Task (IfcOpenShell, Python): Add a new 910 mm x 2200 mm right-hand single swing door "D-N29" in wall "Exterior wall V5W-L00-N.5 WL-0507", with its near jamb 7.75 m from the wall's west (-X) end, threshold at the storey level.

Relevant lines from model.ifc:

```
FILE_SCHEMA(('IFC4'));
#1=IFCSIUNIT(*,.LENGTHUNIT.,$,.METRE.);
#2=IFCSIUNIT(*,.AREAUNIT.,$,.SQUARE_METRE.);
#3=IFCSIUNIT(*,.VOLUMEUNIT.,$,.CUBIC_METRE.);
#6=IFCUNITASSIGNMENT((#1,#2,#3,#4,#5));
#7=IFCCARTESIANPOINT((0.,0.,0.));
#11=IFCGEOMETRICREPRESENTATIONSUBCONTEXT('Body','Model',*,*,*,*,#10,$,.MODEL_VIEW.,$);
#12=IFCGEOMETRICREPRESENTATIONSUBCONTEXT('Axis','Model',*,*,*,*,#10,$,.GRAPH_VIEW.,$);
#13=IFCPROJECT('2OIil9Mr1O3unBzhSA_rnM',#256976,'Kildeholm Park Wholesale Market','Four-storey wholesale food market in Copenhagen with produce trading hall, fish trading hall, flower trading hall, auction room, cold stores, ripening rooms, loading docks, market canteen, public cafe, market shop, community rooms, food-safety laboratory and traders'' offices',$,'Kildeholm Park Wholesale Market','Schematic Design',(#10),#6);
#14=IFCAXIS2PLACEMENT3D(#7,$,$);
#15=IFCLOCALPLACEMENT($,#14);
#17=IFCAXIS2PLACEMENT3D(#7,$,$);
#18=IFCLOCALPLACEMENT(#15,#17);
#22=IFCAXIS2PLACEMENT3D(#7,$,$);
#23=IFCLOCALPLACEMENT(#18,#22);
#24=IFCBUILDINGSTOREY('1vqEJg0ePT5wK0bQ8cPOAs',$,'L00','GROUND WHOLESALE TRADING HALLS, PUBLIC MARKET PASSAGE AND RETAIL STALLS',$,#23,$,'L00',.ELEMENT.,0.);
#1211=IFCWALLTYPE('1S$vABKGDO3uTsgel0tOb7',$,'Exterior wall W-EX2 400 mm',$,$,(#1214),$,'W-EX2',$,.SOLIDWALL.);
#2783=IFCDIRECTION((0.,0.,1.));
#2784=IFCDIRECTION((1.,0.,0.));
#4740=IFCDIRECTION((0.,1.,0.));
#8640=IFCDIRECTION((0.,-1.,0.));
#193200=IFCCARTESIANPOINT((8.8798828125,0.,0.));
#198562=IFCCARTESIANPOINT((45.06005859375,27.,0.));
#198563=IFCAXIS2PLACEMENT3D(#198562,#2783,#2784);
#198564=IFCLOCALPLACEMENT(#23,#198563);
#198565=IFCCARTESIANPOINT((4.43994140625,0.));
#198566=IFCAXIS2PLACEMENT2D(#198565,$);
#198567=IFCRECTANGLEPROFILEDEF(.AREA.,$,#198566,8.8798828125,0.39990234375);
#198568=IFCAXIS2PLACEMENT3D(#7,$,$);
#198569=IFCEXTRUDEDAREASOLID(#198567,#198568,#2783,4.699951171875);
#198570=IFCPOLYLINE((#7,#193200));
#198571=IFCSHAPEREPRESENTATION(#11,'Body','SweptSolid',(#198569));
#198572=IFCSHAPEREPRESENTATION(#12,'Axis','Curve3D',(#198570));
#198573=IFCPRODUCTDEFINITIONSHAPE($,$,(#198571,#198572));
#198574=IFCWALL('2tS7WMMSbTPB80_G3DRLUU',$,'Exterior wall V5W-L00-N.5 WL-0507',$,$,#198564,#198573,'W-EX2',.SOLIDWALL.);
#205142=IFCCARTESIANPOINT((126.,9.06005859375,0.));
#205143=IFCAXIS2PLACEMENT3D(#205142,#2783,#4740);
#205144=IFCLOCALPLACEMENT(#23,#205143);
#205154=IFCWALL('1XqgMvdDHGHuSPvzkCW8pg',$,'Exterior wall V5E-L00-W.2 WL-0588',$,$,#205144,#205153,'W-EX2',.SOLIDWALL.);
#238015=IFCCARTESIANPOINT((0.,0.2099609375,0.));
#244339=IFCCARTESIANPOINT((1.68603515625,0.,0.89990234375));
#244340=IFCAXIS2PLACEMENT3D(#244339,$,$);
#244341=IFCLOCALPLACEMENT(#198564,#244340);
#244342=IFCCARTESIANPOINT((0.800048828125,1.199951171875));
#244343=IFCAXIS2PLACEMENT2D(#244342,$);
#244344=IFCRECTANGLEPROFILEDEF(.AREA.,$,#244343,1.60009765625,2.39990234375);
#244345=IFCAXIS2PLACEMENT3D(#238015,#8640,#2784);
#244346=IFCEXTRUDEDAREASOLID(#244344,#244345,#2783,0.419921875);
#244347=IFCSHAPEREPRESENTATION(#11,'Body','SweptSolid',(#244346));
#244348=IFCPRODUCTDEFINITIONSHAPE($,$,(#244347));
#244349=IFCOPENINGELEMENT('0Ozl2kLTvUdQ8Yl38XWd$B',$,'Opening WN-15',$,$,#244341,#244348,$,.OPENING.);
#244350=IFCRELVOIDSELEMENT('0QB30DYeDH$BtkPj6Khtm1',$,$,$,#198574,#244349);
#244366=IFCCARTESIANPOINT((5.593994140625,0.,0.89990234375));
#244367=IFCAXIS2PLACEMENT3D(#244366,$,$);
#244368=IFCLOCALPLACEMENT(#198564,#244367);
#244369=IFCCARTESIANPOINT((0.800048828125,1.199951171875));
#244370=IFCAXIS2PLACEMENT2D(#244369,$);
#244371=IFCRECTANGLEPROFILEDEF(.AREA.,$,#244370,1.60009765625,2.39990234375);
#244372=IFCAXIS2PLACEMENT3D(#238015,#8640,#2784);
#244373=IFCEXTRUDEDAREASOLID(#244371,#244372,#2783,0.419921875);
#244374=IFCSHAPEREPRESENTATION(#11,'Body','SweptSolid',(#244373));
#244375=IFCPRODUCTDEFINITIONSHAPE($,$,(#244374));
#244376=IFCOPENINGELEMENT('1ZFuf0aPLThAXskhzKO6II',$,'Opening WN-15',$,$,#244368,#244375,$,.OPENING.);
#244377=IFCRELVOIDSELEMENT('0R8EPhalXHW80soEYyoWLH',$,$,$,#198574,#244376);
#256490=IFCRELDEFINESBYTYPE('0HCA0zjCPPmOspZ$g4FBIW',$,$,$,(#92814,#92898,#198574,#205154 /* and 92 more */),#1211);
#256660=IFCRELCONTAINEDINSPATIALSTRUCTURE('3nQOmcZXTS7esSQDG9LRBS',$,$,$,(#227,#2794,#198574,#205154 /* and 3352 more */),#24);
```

```python
import numpy as np
import ifcopenshell
import ifcopenshell.api.feature
import ifcopenshell.api.geometry
import ifcopenshell.api.root
import ifcopenshell.api.spatial
import ifcopenshell.geom
import ifcopenshell.util.element
import ifcopenshell.util.placement
import ifcopenshell.util.representation
import ifcopenshell.util.shape
import ifcopenshell.util.unit

model = ifcopenshell.open("model.ifc")
unit_scale = ifcopenshell.util.unit.calculate_unit_scale(model)
settings = ifcopenshell.geom.settings()


def volume(element):
    """Net volume in cubic metres, openings subtracted."""
    shape = ifcopenshell.geom.create_shape(settings, element)
    return ifcopenshell.util.shape.get_volume(shape.geometry)


wall = model.by_guid("2tS7WMMSbTPB80_G3DRLUU")
storey = ifcopenshell.util.element.get_container(wall, ifc_class="IfcBuildingStorey")
context = ifcopenshell.util.representation.get_context(model, "Model", "Body", "MODEL_VIEW")
before = volume(wall)

width, height, from_end, sill = 0.91, 2.2, 7.75, 0.0  # metres

# The wall runs along its own X axis, and the end named is its -X end.
wall_shape = ifcopenshell.geom.create_shape(settings, wall)
x, y, z = ifcopenshell.util.shape.get_vertices(wall_shape.geometry).T
start = x.min() + from_end
face, thickness = float(y.min()), float(y.max() - y.min())
wall_matrix = ifcopenshell.util.placement.get_local_placement(wall.ObjectPlacement)
level = ifcopenshell.util.placement.get_local_placement(storey.ObjectPlacement)[2, 3]


def in_wall(x, y):
    """Placement at x, y metres in the wall's axes, at sill height."""
    matrix = wall_matrix.copy()
    matrix[:, 3] = wall_matrix @ np.array([x / unit_scale, y / unit_scale, 0.0, 1.0])
    matrix[2, 3] = level + sill / unit_scale
    return matrix


# Opening: a box that overshoots both wall faces by 50 mm.
opening = ifcopenshell.api.root.create_entity(model, ifc_class="IfcOpeningElement", predefined_type="OPENING")
box = ifcopenshell.api.geometry.add_wall_representation(
    model, context=context, length=width, height=height, thickness=thickness + 0.1
)
ifcopenshell.api.geometry.assign_representation(model, product=opening, representation=box)
ifcopenshell.api.geometry.edit_object_placement(model, product=opening, matrix=in_wall(start, face - 0.05), is_si=False)
ifcopenshell.api.feature.add_feature(model, feature=opening, element=wall)

door = ifcopenshell.api.root.create_entity(model, ifc_class="IfcDoor", name="D-N29", predefined_type="DOOR")
door.OverallWidth, door.OverallHeight = width / unit_scale, height / unit_scale
door.OperationType = "SINGLE_SWING_RIGHT"
body = ifcopenshell.api.geometry.add_door_representation(
    model,
    context=context,
    overall_width=door.OverallWidth,
    overall_height=door.OverallHeight,
    operation_type="SINGLE_SWING_RIGHT",
    lining_properties={"LiningDepth": thickness / unit_scale, "ThresholdDepth": thickness / unit_scale},
)
ifcopenshell.api.geometry.assign_representation(model, product=door, representation=body)
ifcopenshell.api.spatial.assign_container(model, products=[door], relating_structure=storey)
ifcopenshell.api.feature.add_filling(model, opening=opening, element=door)

# The lining spans the wall, so the door starts at the wall face.
ifcopenshell.api.geometry.edit_object_placement(model, product=door, matrix=in_wall(start, face), is_si=False)

after = volume(wall)

print(f"wall volume {before:.3f} -> {after:.3f} m3")

model.write("model_edited.ifc")
```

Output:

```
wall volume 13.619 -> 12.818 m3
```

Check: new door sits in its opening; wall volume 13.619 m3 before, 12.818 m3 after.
